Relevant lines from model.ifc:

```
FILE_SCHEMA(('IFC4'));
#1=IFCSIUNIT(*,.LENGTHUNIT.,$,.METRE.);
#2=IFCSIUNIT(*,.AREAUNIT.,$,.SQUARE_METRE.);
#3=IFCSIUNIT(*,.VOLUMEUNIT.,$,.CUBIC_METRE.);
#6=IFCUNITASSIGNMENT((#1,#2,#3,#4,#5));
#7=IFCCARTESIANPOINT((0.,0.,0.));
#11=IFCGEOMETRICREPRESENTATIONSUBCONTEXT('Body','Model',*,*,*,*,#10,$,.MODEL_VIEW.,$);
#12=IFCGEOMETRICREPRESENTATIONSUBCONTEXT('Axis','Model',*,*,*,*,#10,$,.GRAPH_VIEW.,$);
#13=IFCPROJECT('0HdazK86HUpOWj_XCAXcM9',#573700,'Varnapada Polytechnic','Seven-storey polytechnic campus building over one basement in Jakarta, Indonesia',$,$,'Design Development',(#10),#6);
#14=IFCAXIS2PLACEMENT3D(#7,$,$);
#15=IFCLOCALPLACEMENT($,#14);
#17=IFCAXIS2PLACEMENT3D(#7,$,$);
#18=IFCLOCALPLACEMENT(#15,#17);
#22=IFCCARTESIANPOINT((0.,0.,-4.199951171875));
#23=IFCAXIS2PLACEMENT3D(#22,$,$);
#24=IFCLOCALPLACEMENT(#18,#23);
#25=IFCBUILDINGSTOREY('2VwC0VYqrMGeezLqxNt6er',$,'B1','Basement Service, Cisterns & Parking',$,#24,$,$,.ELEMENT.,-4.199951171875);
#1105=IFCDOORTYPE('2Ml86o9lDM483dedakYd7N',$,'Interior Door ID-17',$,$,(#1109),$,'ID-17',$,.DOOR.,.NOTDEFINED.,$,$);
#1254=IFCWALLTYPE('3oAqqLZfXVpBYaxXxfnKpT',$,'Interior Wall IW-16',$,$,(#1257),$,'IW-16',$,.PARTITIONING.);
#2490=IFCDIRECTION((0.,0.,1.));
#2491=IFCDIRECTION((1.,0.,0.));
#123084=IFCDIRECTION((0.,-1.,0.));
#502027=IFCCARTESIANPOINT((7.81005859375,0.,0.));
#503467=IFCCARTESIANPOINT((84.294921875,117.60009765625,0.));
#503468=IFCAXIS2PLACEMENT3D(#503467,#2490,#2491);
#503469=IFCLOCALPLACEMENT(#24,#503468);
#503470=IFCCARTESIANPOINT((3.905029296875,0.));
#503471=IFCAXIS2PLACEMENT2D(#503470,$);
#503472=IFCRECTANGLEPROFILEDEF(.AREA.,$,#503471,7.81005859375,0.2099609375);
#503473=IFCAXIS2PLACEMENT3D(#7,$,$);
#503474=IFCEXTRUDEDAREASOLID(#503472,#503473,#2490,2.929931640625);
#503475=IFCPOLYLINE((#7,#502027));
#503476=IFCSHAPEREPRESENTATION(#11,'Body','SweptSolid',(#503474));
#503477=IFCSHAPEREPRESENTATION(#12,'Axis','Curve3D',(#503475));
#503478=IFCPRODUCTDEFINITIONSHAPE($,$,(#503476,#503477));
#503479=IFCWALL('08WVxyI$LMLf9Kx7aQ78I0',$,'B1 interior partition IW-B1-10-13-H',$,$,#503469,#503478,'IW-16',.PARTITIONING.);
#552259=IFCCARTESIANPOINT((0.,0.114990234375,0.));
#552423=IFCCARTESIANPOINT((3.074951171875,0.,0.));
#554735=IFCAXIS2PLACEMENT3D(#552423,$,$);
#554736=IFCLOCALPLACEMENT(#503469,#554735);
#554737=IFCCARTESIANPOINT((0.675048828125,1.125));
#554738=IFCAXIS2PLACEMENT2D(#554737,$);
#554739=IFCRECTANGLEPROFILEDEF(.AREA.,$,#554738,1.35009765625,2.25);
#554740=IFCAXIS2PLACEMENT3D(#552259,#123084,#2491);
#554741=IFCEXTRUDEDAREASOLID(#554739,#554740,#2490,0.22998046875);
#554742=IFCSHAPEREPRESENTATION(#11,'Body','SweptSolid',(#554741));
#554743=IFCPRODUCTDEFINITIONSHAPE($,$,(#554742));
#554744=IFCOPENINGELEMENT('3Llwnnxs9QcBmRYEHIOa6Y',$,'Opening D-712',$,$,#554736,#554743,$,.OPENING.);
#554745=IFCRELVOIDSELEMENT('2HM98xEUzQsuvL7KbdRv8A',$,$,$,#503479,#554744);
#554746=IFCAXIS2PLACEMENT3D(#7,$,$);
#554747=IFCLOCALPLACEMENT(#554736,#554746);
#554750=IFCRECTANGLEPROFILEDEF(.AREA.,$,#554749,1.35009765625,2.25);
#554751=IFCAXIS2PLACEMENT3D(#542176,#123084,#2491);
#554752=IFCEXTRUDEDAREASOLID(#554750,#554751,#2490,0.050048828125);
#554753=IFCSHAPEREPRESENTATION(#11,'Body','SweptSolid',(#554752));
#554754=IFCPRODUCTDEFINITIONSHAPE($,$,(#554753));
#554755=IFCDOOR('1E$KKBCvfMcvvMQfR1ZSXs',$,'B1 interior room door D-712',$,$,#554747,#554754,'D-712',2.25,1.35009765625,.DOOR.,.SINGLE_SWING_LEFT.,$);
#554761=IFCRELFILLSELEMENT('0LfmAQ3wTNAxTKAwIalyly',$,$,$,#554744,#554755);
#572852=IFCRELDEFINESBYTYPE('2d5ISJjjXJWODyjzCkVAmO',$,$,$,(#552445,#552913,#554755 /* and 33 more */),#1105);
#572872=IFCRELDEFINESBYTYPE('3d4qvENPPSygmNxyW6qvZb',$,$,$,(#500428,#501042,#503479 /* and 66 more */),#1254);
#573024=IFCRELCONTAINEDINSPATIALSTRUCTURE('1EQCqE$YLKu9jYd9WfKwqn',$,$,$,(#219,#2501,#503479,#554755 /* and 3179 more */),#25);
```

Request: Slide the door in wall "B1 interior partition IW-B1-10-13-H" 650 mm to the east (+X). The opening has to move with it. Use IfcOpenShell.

```python
import ifcopenshell
import ifcopenshell.api.geometry
import ifcopenshell.util.placement
import ifcopenshell.util.unit

model = ifcopenshell.open("model.ifc")
unit_scale = ifcopenshell.util.unit.calculate_unit_scale(model)

door = model.by_guid("1E$KKBCvfMcvvMQfR1ZSXs")
opening = door.FillsVoids[0].RelatingOpeningElement
wall = opening.VoidsElements[0].RelatingBuildingElement

wall_matrix = ifcopenshell.util.placement.get_local_placement(wall.ObjectPlacement)
shift = wall_matrix[:3, 0] * 0.65 / unit_scale
before = ifcopenshell.util.placement.get_local_placement(door.ObjectPlacement)[:3, 3].copy()

# The door is placed relative to its opening, so it follows when the opening moves.
matrix = ifcopenshell.util.placement.get_local_placement(opening.ObjectPlacement)
matrix[:3, 3] += shift
ifcopenshell.api.geometry.edit_object_placement(
    model, product=opening, matrix=matrix, is_si=False, should_transform_children=True
)

after = ifcopenshell.util.placement.get_local_placement(door.ObjectPlacement)[:3, 3]
print("door moved by", (after - before).round(3) + 0.0)

model.write("model_v2.ifc")
```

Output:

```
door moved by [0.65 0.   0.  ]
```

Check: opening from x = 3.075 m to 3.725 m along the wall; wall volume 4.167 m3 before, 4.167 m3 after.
